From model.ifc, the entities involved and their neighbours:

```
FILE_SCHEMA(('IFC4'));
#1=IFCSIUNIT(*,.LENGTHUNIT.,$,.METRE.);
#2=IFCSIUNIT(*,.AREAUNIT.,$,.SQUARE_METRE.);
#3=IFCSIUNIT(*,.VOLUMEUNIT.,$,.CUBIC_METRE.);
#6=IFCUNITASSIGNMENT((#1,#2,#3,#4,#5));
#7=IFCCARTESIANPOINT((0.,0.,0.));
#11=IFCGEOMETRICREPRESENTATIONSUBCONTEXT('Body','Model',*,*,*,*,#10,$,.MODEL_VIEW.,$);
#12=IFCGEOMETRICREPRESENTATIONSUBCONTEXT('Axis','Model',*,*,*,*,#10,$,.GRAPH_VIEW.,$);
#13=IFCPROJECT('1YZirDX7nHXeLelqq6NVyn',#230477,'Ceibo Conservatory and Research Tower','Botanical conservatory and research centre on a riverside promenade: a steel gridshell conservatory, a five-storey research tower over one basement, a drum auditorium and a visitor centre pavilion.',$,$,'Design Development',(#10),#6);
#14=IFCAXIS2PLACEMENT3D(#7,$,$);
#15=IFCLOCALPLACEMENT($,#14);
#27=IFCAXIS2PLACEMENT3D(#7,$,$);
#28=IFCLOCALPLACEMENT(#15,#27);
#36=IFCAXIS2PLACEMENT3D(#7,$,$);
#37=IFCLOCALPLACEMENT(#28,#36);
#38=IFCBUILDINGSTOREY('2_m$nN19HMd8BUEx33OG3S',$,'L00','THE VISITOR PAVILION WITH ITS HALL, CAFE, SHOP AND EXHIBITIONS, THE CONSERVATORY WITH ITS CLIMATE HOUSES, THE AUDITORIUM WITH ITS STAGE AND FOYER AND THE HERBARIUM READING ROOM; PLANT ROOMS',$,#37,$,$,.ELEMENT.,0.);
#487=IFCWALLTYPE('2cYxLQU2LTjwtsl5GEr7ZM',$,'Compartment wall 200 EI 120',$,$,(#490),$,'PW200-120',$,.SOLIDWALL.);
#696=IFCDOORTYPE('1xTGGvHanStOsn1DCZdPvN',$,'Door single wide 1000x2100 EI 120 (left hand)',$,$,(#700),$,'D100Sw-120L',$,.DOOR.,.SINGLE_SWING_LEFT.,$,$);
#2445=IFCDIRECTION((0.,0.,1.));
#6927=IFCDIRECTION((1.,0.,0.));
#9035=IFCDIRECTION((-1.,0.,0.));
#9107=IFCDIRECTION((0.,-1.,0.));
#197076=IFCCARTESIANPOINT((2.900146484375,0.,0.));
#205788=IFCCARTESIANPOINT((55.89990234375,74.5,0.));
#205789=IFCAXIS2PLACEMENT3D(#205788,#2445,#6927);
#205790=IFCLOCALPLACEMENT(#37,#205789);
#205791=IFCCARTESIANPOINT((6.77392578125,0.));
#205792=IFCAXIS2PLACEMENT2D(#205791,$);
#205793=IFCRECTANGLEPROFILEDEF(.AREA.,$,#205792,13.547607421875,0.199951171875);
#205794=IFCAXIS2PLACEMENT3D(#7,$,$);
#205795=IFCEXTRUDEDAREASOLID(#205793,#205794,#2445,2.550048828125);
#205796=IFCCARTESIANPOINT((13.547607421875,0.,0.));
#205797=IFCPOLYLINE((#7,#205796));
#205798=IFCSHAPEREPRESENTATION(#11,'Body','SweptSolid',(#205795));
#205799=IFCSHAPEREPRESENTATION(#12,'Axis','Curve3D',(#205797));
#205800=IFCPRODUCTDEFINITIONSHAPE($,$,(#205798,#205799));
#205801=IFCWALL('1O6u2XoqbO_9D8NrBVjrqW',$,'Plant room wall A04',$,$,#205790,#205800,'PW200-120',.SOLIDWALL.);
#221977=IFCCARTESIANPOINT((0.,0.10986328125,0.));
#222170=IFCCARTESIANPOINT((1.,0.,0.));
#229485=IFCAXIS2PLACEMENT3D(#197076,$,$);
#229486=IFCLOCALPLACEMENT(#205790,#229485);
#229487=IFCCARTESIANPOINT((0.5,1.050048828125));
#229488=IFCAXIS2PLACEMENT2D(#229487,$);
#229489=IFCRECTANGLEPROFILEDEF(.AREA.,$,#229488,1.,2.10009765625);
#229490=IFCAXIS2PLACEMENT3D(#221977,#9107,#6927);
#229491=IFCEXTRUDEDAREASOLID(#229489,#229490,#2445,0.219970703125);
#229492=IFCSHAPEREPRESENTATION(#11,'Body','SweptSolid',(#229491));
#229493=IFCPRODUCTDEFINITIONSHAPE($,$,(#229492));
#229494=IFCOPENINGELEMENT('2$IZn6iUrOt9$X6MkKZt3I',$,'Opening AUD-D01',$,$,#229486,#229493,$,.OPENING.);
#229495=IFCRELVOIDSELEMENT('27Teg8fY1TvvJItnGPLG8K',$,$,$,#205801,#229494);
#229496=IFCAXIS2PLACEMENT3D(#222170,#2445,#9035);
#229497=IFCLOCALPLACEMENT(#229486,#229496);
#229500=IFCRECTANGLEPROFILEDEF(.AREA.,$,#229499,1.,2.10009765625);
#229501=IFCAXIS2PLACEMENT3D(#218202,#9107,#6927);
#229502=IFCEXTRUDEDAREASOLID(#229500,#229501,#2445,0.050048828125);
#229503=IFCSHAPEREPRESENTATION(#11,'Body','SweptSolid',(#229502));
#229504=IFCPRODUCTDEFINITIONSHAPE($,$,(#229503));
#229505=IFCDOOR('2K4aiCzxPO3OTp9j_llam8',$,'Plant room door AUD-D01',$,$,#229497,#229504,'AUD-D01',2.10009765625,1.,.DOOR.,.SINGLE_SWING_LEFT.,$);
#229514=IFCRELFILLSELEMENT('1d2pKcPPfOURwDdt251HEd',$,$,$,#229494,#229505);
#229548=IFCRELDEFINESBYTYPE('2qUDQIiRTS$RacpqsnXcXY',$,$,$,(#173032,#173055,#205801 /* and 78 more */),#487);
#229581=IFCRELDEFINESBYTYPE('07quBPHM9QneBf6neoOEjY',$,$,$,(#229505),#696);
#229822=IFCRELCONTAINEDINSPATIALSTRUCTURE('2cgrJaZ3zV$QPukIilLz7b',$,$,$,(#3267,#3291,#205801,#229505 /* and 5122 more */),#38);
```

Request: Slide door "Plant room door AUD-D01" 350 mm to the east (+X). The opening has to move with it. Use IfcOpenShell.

```python
import ifcopenshell
import ifcopenshell.api.geometry
import ifcopenshell.util.placement
import ifcopenshell.util.unit

model = ifcopenshell.open("model.ifc")
unit_scale = ifcopenshell.util.unit.calculate_unit_scale(model)

door = model.by_guid("2K4aiCzxPO3OTp9j_llam8")
opening = door.FillsVoids[0].RelatingOpeningElement
wall = opening.VoidsElements[0].RelatingBuildingElement

wall_matrix = ifcopenshell.util.placement.get_local_placement(wall.ObjectPlacement)
shift = wall_matrix[:3, 0] * 0.35 / unit_scale
before = ifcopenshell.util.placement.get_local_placement(door.ObjectPlacement)[:3, 3].copy()

# The door is placed relative to its opening, so it follows when the opening moves.
matrix = ifcopenshell.util.placement.get_local_placement(opening.ObjectPlacement)
matrix[:3, 3] += shift
ifcopenshell.api.geometry.edit_object_placement(
    model, product=opening, matrix=matrix, is_si=False, should_transform_children=True
)

after = ifcopenshell.util.placement.get_local_placement(door.ObjectPlacement)[:3, 3]
print("door moved by", (after - before).round(3) + 0.0)

model.write("model_edited.ifc")
```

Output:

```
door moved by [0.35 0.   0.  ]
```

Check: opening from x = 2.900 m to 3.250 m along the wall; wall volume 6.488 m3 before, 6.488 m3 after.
